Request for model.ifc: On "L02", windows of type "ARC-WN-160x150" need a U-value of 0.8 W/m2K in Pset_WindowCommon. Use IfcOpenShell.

First a look at what the model holds.

```python
import ifcopenshell
import ifcopenshell.util.element

model = ifcopenshell.open("model.ifc")
print(model.schema)
storey = next(s for s in model.by_type("IfcBuildingStorey") if s.Name == "L02")
windows = [e for e in ifcopenshell.util.element.get_decomposition(storey) if e.is_a("IfcWindow")]
seen = {}
for e in windows:
    element_type = ifcopenshell.util.element.get_type(e)
    key = (element_type.Name if element_type != e and element_type else None, ifcopenshell.util.element.get_pset(e, "Pset_WindowCommon", "ThermalTransmittance"))
    seen[key] = seen.get(key, 0) + 1
for (name, value), count in sorted(seen.items(), key=str):
    print(count, "x", name, "|", value)
```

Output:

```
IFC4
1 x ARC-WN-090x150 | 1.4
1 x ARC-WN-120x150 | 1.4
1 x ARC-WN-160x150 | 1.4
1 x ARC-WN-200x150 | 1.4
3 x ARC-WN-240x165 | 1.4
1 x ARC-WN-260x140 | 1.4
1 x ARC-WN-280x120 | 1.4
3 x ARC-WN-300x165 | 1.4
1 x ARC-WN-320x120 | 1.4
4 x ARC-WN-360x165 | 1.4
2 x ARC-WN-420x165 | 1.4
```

```python
import ifcopenshell
import ifcopenshell.api.pset
import ifcopenshell.util.element

model = ifcopenshell.open("model.ifc")

storey = next(s for s in model.by_type("IfcBuildingStorey") if s.Name == "L02")
windows = [e for e in ifcopenshell.util.element.get_decomposition(storey) if e.is_a("IfcWindow")]

count = 0
for e in windows:
    element_type = ifcopenshell.util.element.get_type(e)
    if element_type in (None, e) or element_type.Name != "ARC-WN-160x150":
        continue
    # add_pset returns the element's existing set when there is one.
    pset = ifcopenshell.api.pset.add_pset(model, product=e, name="Pset_WindowCommon")
    ifcopenshell.api.pset.edit_pset(model, pset=pset, properties={"ThermalTransmittance": 0.8})
    count += 1

print(count, "windows updated")

model.write("model-out.ifc")
```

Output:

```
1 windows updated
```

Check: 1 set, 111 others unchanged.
